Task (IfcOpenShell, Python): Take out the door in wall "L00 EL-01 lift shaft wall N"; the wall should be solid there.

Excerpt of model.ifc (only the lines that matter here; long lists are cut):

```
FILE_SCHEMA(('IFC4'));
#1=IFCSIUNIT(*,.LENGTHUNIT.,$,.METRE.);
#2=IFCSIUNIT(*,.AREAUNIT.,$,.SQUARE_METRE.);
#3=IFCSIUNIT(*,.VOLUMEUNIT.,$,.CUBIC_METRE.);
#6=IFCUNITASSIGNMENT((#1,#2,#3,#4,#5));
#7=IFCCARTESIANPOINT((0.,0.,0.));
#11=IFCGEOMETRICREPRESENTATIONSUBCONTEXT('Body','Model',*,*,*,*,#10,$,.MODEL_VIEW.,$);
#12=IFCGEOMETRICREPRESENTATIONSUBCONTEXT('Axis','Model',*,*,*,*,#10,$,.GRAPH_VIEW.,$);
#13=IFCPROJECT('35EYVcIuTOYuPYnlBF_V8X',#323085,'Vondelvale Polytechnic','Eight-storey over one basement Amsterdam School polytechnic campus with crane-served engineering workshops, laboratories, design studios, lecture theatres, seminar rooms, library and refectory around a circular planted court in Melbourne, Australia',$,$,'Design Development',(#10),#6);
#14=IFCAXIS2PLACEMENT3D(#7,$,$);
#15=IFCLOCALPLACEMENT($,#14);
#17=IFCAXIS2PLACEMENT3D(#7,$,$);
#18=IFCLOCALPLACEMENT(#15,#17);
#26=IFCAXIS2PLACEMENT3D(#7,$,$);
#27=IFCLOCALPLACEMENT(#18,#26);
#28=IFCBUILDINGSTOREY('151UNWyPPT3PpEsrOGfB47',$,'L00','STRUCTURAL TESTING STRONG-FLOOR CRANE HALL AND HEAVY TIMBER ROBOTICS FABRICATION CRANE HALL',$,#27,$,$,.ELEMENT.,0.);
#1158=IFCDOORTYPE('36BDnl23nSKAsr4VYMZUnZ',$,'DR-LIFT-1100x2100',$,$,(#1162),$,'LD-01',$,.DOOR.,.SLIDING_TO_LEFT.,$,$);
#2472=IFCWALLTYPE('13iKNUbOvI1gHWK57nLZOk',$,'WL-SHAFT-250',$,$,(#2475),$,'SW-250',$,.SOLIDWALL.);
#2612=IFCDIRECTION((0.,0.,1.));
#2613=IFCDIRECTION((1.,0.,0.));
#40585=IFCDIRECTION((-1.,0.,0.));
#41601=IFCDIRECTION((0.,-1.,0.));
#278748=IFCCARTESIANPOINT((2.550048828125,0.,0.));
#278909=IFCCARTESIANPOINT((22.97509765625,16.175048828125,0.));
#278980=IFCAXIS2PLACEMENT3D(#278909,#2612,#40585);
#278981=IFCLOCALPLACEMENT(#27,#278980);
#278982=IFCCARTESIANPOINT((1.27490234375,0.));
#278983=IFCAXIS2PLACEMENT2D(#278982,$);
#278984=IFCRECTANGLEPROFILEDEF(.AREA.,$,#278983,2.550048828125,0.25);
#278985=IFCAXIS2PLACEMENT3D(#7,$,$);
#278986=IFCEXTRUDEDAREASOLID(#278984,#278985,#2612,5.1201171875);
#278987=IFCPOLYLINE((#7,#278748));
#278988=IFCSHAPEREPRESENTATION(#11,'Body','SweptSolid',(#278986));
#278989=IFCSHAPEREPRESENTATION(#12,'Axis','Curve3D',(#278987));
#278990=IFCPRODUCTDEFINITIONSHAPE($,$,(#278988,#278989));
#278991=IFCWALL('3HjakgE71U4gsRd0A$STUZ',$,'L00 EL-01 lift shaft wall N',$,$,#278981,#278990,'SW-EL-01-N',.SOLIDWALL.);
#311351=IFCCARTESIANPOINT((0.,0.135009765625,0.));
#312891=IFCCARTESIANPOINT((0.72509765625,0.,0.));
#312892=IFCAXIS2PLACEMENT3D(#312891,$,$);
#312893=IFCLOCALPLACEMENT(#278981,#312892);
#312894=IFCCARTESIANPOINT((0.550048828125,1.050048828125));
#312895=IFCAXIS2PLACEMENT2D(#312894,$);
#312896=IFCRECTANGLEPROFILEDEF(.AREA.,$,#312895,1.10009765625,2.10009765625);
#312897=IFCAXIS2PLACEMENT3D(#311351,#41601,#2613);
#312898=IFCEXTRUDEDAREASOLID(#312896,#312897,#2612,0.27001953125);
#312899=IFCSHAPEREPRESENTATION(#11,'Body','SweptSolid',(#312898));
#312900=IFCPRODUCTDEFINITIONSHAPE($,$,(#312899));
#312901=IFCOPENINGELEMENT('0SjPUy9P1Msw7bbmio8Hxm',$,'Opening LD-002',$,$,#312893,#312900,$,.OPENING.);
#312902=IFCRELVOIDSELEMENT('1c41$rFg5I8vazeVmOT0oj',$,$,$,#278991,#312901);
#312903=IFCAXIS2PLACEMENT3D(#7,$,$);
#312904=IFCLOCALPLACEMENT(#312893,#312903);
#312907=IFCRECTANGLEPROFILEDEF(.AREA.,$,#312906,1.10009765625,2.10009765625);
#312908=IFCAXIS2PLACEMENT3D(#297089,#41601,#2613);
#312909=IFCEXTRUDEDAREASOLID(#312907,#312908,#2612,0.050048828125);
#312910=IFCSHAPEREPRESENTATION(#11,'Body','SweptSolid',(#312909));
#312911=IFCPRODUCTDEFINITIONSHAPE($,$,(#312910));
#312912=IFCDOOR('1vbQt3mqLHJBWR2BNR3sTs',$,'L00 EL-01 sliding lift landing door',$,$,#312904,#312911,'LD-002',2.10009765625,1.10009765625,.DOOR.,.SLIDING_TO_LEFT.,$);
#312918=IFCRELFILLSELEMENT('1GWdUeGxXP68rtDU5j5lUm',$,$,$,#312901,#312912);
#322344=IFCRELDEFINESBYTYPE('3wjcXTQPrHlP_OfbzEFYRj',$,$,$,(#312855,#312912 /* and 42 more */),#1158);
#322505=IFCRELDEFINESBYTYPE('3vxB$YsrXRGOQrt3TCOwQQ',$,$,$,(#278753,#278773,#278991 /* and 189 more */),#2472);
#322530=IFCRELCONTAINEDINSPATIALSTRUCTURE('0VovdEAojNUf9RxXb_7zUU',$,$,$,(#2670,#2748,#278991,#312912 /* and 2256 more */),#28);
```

```python
import ifcopenshell
import ifcopenshell.api.feature
import ifcopenshell.api.root
import ifcopenshell.geom
import ifcopenshell.util.shape

model = ifcopenshell.open("model.ifc")
settings = ifcopenshell.geom.settings()


def volume(element):
    """Net volume in cubic metres, openings subtracted."""
    shape = ifcopenshell.geom.create_shape(settings, element)
    return ifcopenshell.util.shape.get_volume(shape.geometry)


door = model.by_guid("1vbQt3mqLHJBWR2BNR3sTs")
opening = door.FillsVoids[0].RelatingOpeningElement
wall = opening.VoidsElements[0].RelatingBuildingElement
before = volume(wall)

ifcopenshell.api.root.remove_product(model, product=door)
ifcopenshell.api.feature.remove_feature(model, feature=opening)

after = volume(wall)

print(f"wall volume {before:.3f} -> {after:.3f} m3")

model.write("model_updated.ifc")
```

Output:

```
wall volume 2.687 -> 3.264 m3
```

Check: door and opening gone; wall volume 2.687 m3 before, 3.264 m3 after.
